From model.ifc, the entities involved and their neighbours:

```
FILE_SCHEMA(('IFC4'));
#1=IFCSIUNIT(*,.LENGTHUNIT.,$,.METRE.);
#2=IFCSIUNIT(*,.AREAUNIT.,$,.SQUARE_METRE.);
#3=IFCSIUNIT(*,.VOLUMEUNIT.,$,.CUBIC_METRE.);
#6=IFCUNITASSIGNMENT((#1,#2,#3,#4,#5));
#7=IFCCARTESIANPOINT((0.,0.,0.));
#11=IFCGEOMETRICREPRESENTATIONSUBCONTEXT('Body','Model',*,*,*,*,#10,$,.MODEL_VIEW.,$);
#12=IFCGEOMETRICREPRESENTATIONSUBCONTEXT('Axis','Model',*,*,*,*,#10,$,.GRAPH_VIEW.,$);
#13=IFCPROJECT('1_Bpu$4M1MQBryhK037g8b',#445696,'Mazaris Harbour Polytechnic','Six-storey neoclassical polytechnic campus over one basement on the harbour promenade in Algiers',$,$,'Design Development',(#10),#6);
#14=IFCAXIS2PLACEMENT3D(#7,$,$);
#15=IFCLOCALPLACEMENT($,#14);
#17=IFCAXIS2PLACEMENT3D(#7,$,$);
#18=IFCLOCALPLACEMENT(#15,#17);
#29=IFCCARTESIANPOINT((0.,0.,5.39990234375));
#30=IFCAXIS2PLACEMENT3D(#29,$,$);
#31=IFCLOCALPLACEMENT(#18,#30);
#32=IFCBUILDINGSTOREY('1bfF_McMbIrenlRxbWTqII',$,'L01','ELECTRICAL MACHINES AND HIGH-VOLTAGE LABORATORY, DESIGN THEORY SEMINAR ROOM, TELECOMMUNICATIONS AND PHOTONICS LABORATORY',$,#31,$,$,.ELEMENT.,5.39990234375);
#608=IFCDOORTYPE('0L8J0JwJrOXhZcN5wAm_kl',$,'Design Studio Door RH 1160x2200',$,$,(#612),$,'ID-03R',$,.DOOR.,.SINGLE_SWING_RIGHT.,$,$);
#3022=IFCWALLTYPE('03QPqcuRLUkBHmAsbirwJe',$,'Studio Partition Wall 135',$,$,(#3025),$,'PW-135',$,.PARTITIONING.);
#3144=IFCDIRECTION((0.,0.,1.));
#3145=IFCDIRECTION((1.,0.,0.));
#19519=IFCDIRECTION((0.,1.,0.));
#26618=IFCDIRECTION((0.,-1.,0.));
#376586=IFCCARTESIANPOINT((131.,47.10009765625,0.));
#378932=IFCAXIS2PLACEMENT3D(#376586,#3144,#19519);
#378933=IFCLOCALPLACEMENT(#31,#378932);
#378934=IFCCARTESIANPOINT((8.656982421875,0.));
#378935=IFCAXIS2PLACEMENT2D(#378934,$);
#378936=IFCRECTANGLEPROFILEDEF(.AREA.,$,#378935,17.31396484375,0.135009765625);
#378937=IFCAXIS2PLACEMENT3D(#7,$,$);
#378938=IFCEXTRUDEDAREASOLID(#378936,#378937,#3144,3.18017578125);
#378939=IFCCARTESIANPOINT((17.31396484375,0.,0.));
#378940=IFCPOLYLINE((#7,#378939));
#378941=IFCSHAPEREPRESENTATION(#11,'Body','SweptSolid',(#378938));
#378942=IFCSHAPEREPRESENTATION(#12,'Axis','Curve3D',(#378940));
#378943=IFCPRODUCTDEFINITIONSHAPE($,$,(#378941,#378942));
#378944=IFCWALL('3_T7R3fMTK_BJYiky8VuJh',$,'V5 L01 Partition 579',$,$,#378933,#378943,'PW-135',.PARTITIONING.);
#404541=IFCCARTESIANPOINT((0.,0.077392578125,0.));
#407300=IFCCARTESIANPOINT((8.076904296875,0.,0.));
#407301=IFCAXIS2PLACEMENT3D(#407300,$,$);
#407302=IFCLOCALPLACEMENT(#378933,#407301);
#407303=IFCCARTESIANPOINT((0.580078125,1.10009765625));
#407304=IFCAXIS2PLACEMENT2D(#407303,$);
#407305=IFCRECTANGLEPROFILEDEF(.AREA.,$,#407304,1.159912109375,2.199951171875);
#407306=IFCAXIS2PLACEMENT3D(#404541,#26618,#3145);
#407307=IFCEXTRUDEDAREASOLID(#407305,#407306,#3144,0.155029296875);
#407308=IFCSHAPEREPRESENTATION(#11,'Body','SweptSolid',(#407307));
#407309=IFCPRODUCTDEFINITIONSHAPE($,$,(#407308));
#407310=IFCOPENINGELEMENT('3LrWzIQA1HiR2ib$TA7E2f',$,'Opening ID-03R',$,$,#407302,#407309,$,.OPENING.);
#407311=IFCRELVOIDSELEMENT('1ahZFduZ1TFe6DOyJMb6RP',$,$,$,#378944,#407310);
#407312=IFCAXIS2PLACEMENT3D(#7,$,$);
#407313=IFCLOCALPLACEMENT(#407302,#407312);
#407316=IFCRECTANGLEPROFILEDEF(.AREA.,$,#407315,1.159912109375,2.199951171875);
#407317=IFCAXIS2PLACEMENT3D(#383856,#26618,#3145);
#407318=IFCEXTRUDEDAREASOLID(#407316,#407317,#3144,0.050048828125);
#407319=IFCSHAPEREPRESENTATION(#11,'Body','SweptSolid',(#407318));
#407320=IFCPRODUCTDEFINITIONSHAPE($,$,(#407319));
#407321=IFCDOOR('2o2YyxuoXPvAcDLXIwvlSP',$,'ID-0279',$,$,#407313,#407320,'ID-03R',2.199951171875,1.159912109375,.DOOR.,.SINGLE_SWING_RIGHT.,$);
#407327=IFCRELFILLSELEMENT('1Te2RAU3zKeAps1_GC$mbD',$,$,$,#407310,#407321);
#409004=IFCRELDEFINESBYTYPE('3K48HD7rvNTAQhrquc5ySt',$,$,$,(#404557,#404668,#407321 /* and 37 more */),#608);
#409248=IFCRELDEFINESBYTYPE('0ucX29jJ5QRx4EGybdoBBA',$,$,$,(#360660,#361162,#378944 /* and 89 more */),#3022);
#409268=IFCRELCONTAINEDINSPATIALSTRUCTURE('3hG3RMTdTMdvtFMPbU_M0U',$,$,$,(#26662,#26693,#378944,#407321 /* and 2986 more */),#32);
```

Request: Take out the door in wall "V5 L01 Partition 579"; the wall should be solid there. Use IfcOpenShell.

```python
import ifcopenshell
import ifcopenshell.api.feature
import ifcopenshell.api.root
import ifcopenshell.geom
import ifcopenshell.util.shape

model = ifcopenshell.open("model.ifc")
settings = ifcopenshell.geom.settings()


def volume(element):
    """Net volume in cubic metres, openings subtracted."""
    shape = ifcopenshell.geom.create_shape(settings, element)
    return ifcopenshell.util.shape.get_volume(shape.geometry)


door = model.by_id(407321)
opening = door.FillsVoids[0].RelatingOpeningElement
wall = opening.VoidsElements[0].RelatingBuildingElement
before = volume(wall)

ifcopenshell.api.root.remove_product(model, product=door)
ifcopenshell.api.feature.remove_feature(model, feature=opening)

after = volume(wall)

print(f"wall volume {before:.3f} -> {after:.3f} m3")

model.write("model-out.ifc")
```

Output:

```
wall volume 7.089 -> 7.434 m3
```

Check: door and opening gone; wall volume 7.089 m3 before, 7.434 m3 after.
